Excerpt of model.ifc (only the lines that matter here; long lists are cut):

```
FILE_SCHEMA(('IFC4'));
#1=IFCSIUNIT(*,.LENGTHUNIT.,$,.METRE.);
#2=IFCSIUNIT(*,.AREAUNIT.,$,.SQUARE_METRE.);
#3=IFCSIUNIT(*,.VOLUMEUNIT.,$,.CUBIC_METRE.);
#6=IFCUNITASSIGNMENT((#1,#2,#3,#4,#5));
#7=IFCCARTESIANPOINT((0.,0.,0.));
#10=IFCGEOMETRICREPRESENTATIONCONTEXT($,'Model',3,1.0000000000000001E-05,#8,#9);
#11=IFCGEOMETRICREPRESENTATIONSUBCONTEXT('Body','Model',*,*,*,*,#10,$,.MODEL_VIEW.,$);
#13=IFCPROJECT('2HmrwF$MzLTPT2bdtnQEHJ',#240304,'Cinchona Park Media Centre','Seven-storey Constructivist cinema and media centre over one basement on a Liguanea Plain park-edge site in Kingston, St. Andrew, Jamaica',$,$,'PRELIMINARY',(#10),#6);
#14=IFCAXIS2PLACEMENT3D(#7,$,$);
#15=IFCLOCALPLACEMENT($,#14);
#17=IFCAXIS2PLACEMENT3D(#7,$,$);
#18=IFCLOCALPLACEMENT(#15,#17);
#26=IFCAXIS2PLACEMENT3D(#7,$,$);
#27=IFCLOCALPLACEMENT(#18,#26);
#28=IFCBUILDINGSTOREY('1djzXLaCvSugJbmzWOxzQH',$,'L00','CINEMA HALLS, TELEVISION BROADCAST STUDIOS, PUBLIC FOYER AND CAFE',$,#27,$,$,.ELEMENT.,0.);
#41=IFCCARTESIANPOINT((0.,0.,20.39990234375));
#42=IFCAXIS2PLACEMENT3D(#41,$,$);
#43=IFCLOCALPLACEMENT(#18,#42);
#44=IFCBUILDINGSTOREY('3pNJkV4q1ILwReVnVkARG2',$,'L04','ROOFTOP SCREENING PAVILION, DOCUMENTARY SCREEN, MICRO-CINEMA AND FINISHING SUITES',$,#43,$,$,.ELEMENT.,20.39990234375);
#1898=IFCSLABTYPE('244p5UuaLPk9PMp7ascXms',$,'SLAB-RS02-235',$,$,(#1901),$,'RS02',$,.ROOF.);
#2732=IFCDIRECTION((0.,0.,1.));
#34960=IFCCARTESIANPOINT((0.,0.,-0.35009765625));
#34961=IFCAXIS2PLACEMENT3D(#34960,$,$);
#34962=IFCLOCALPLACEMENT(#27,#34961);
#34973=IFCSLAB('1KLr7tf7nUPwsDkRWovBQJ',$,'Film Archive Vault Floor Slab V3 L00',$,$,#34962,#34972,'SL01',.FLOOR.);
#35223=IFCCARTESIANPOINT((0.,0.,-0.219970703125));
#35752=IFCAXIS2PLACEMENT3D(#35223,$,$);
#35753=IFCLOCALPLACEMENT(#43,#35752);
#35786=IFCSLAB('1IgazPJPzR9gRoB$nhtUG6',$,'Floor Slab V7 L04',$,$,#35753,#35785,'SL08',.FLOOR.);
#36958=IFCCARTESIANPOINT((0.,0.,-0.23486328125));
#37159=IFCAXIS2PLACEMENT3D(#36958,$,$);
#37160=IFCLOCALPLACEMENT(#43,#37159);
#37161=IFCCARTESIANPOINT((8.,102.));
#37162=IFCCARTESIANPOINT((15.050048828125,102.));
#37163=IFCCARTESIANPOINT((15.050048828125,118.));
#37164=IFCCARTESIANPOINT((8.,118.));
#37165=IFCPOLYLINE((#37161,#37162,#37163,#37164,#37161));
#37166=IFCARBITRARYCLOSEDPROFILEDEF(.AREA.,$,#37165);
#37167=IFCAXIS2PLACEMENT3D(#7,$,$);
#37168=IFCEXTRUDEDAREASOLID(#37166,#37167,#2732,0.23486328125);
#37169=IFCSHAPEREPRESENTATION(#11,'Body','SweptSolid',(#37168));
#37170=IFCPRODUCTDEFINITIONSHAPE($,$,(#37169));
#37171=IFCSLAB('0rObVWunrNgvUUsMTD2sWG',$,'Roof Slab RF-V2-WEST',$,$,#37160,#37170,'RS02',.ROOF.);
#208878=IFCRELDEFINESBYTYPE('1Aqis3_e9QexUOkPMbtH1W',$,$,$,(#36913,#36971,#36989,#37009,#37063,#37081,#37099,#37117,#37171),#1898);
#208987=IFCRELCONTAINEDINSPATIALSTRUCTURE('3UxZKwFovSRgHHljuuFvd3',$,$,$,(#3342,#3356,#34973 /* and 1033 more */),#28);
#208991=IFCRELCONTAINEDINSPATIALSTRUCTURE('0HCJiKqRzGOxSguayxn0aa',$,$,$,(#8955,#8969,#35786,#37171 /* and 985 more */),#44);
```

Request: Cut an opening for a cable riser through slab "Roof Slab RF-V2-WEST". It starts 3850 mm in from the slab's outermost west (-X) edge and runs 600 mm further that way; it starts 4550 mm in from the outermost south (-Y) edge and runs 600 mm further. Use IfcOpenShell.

```python
import numpy as np
import ifcopenshell
import ifcopenshell.api.feature
import ifcopenshell.api.geometry
import ifcopenshell.api.root
import ifcopenshell.geom
import ifcopenshell.util.placement
import ifcopenshell.util.representation
import ifcopenshell.util.shape
import ifcopenshell.util.unit

model = ifcopenshell.open("model.ifc")
unit_scale = ifcopenshell.util.unit.calculate_unit_scale(model)
settings = ifcopenshell.geom.settings()


def volume(element):
    """Net volume in cubic metres, openings subtracted."""
    shape = ifcopenshell.geom.create_shape(settings, element)
    return ifcopenshell.util.shape.get_volume(shape.geometry)


slab = model.by_guid("0rObVWunrNgvUUsMTD2sWG")
before = volume(slab)

# Extent in the slab's own axes, in metres. The edges named are its -X and -Y sides.
slab_shape = ifcopenshell.geom.create_shape(settings, slab)
vertices = ifcopenshell.util.shape.get_vertices(slab_shape.geometry)
x_min, y_min, bottom = vertices.min(axis=0)
top = vertices[:, 2].max()

opening = ifcopenshell.api.root.create_entity(model, ifc_class="IfcOpeningElement", name="Cable riser opening", predefined_type="OPENING")
context = ifcopenshell.util.representation.get_context(model, "Model", "Body", "MODEL_VIEW")
width, depth = 0.6, 0.6
outline = [(0.0, 0.0), (width, 0.0), (width, depth), (0.0, depth), (0.0, 0.0)]
# Overshoot both faces by 50 mm so the cut is clean.
shape = ifcopenshell.api.geometry.add_slab_representation(
    model, context=context, depth=top - bottom + 0.1, polyline=outline
)
ifcopenshell.api.geometry.assign_representation(model, product=opening, representation=shape)

matrix = ifcopenshell.util.placement.get_local_placement(slab.ObjectPlacement)
matrix[:, 3] = matrix @ np.append(np.array([x_min + 3.85, y_min + 4.55, bottom - 0.05]) / unit_scale, 1.0)
ifcopenshell.api.geometry.edit_object_placement(model, product=opening, matrix=matrix, is_si=False)
ifcopenshell.api.feature.add_feature(model, feature=opening, element=slab)

after = volume(slab)

print(f"slab volume {before:.3f} -> {after:.3f} m3")

model.write("model_rev.ifc")
```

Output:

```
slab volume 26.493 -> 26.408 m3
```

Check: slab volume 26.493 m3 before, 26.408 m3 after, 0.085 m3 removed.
